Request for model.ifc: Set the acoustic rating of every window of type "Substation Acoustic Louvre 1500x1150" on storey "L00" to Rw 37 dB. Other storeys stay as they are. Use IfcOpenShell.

First a look at what the model holds.

```python
import ifcopenshell
import ifcopenshell.util.element

model = ifcopenshell.open("model.ifc")
print(model.schema)
storey = next(s for s in model.by_type("IfcBuildingStorey") if s.Name == "L00")
windows = [e for e in ifcopenshell.util.element.get_decomposition(storey) if e.is_a("IfcWindow")]
seen = {}
for e in windows:
    element_type = ifcopenshell.util.element.get_type(e)
    key = (element_type.Name if element_type != e and element_type else None, ifcopenshell.util.element.get_pset(e, "Pset_WindowCommon", "AcousticRating"))
    seen[key] = seen.get(key, 0) + 1
for (name, value), count in sorted(seen.items(), key=str):
    print(count, "x", name, "|", value)
```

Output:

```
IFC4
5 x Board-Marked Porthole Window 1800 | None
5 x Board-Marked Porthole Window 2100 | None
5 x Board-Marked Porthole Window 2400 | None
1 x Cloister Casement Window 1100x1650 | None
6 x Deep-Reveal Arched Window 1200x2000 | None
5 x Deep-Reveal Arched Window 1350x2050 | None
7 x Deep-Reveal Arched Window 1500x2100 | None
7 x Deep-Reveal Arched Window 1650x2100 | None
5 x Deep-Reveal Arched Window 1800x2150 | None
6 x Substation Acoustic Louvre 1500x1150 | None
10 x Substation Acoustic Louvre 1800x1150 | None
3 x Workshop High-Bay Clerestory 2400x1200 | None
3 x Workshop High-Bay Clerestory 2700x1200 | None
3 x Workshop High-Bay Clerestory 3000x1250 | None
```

```python
import ifcopenshell
import ifcopenshell.api.pset
import ifcopenshell.util.element

model = ifcopenshell.open("model.ifc")

storey = next(s for s in model.by_type("IfcBuildingStorey") if s.Name == "L00")
windows = [e for e in ifcopenshell.util.element.get_decomposition(storey) if e.is_a("IfcWindow")]

count = 0
for e in windows:
    element_type = ifcopenshell.util.element.get_type(e)
    if element_type in (None, e) or element_type.Name != "Substation Acoustic Louvre 1500x1150":
        continue
    # add_pset returns the element's existing set when there is one.
    pset = ifcopenshell.api.pset.add_pset(model, product=e, name="Pset_WindowCommon")
    ifcopenshell.api.pset.edit_pset(model, pset=pset, properties={"AcousticRating": "Rw 37 dB"})
    count += 1

print(count, "windows updated")

model.write("model_edited.ifc")
```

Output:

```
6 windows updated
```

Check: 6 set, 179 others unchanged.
